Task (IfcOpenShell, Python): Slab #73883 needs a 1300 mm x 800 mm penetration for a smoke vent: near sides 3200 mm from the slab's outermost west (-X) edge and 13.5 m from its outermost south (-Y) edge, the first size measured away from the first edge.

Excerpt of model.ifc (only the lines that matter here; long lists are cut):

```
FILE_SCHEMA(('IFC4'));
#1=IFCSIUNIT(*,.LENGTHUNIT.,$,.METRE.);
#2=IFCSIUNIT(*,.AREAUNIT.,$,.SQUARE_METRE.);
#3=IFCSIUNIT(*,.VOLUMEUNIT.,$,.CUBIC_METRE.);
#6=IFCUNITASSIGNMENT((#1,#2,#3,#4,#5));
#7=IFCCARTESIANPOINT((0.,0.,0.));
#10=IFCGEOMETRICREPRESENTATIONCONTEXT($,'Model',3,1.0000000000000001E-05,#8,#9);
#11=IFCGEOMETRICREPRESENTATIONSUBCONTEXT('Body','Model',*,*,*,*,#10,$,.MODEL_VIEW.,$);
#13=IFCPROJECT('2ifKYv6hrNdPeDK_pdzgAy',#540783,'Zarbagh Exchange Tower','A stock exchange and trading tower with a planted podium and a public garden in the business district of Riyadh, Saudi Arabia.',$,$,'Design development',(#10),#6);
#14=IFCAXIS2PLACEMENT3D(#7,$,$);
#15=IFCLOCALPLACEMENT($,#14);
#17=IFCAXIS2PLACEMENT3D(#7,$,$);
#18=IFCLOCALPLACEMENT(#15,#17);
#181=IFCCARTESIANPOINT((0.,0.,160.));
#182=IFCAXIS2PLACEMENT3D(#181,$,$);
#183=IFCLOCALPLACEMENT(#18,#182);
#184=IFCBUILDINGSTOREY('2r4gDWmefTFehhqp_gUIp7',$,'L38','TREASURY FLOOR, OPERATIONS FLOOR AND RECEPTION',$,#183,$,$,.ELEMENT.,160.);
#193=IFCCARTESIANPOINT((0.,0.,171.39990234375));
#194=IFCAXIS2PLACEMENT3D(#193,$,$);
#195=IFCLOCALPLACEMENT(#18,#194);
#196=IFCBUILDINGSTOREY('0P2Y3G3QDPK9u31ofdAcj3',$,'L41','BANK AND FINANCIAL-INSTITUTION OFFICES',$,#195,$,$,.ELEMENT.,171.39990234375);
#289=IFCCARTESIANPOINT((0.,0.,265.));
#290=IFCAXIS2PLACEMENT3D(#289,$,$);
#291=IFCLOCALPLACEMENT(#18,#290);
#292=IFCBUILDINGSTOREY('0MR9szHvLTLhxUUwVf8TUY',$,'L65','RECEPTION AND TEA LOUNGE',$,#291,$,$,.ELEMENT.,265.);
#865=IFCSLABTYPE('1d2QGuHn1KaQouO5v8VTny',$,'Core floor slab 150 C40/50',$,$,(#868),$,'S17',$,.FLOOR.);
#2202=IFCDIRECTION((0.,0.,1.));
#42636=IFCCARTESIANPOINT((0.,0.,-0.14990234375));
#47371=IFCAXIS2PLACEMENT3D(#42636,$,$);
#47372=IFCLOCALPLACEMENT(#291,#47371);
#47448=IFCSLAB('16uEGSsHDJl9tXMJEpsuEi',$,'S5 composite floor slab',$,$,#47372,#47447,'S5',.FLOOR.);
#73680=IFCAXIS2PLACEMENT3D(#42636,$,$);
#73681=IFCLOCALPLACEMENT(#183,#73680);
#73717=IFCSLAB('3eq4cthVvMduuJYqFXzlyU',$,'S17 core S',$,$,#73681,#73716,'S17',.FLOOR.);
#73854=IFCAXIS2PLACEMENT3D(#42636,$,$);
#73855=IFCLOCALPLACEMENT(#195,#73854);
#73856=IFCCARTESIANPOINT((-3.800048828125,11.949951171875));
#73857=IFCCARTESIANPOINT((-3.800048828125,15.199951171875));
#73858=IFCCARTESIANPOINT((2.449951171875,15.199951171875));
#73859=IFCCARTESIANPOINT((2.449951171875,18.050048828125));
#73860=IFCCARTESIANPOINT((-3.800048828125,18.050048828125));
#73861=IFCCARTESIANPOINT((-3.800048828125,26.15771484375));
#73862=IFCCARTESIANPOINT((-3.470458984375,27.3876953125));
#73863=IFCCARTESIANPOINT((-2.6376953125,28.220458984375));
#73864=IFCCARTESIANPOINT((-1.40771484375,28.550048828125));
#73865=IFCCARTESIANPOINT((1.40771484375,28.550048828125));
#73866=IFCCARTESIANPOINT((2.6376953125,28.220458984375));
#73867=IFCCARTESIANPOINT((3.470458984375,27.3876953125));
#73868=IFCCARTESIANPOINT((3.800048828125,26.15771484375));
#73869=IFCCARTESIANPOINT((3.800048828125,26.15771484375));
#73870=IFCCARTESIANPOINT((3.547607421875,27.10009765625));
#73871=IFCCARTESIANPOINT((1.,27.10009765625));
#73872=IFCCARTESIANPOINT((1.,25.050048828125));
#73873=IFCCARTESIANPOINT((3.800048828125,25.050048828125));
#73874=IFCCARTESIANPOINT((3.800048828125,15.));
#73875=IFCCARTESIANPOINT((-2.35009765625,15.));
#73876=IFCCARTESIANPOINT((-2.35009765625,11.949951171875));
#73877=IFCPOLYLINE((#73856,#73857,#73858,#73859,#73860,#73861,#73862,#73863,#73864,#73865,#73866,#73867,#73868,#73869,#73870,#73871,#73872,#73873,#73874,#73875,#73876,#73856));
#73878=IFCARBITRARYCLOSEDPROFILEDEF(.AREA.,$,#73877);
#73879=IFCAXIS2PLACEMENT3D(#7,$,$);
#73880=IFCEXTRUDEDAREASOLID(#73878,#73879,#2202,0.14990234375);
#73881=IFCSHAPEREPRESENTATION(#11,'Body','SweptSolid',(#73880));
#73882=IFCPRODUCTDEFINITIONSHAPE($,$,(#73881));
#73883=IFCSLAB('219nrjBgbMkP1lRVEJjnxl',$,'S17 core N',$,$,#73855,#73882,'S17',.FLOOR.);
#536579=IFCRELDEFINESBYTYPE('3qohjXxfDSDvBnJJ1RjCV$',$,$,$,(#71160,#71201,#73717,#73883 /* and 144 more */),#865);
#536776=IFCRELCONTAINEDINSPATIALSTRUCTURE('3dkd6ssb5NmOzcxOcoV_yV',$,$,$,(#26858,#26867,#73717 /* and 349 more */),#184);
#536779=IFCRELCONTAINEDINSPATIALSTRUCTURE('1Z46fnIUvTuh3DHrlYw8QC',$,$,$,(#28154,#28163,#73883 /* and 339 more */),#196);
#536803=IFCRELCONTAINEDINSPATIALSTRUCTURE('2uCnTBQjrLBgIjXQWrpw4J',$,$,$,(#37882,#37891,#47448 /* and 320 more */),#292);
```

```python
import numpy as np
import ifcopenshell
import ifcopenshell.api.feature
import ifcopenshell.api.geometry
import ifcopenshell.api.root
import ifcopenshell.geom
import ifcopenshell.util.placement
import ifcopenshell.util.representation
import ifcopenshell.util.shape
import ifcopenshell.util.unit

model = ifcopenshell.open("model.ifc")
unit_scale = ifcopenshell.util.unit.calculate_unit_scale(model)
settings = ifcopenshell.geom.settings()


def volume(element):
    """Net volume in cubic metres, openings subtracted."""
    shape = ifcopenshell.geom.create_shape(settings, element)
    return ifcopenshell.util.shape.get_volume(shape.geometry)


slab = model.by_id(73883)
before = volume(slab)

# Extent in the slab's own axes, in metres. The edges named are its -X and -Y sides.
slab_shape = ifcopenshell.geom.create_shape(settings, slab)
vertices = ifcopenshell.util.shape.get_vertices(slab_shape.geometry)
x_min, y_min, bottom = vertices.min(axis=0)
top = vertices[:, 2].max()

opening = ifcopenshell.api.root.create_entity(model, ifc_class="IfcOpeningElement", name="Smoke vent opening", predefined_type="OPENING")
context = ifcopenshell.util.representation.get_context(model, "Model", "Body", "MODEL_VIEW")
width, depth = 1.3, 0.8
outline = [(0.0, 0.0), (width, 0.0), (width, depth), (0.0, depth), (0.0, 0.0)]
# Overshoot both faces by 50 mm so the cut is clean.
shape = ifcopenshell.api.geometry.add_slab_representation(
    model, context=context, depth=top - bottom + 0.1, polyline=outline
)
ifcopenshell.api.geometry.assign_representation(model, product=opening, representation=shape)

matrix = ifcopenshell.util.placement.get_local_placement(slab.ObjectPlacement)
matrix[:, 3] = matrix @ np.append(np.array([x_min + 3.2, y_min + 13.5, bottom - 0.05]) / unit_scale, 1.0)
ifcopenshell.api.geometry.edit_object_placement(model, product=opening, matrix=matrix, is_si=False)
ifcopenshell.api.feature.add_feature(model, feature=opening, element=slab)

after = volume(slab)

print(f"slab volume {before:.3f} -> {after:.3f} m3")

model.write("model_updated.ifc")
```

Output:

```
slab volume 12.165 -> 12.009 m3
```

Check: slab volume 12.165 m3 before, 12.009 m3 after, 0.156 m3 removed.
